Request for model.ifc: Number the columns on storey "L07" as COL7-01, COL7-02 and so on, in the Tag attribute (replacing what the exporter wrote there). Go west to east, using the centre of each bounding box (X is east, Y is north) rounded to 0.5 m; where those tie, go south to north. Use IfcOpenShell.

First a look at what the model holds.

```python
import ifcopenshell
import ifcopenshell.util.element
import ifcopenshell.util.placement

model = ifcopenshell.open("model.ifc")
print(model.schema)
storey = next(s for s in model.by_type("IfcBuildingStorey") if s.Name == "L07")
columns = [e for e in ifcopenshell.util.element.get_decomposition(storey) if e.is_a("IfcColumn")]
for e in sorted(columns, key=lambda e: e.id()):
    origin = ifcopenshell.util.placement.get_local_placement(e.ObjectPlacement)[:3, 3]
    print(e.id(), e.Tag, e.Name, origin.round(2) + 0.0, sep=" | ")
```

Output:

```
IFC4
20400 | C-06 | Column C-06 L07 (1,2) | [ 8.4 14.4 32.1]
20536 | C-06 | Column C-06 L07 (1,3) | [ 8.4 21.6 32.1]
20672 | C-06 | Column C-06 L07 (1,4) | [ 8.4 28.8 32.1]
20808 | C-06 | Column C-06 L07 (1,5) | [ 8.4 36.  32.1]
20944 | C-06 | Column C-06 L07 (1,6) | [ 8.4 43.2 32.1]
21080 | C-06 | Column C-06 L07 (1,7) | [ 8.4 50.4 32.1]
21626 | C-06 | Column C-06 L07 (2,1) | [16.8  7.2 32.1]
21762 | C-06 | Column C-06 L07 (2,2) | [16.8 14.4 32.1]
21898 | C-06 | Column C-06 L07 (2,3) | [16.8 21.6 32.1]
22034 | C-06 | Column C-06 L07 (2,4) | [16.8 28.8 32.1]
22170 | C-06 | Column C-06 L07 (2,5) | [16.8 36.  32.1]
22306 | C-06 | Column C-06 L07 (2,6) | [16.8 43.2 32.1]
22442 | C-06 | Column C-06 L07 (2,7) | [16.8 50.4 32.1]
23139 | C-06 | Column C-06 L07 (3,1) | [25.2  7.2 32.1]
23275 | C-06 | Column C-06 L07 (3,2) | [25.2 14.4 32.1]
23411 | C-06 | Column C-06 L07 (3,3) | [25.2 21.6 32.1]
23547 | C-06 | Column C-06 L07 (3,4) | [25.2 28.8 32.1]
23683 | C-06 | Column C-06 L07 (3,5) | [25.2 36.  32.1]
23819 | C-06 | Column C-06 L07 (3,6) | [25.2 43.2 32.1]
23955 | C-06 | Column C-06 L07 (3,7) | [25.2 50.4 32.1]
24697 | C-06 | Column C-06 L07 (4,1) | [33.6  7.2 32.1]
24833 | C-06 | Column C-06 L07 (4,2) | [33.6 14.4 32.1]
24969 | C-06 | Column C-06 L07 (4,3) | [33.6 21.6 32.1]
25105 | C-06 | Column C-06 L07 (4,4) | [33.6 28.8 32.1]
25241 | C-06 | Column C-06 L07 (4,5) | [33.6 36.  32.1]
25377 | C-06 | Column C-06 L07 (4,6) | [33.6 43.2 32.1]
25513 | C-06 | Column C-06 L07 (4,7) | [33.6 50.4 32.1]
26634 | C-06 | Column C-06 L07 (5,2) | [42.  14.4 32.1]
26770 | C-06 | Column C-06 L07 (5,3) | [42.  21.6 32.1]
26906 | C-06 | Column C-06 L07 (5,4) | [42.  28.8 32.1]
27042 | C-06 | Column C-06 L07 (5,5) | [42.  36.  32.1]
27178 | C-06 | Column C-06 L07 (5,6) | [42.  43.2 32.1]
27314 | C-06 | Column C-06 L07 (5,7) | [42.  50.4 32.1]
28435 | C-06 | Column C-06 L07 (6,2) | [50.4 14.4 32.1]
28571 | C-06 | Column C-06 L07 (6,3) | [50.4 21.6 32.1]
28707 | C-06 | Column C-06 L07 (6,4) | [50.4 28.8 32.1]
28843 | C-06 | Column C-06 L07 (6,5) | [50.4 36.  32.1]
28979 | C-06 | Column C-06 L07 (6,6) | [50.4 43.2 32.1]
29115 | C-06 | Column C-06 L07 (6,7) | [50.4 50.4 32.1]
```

```python
import ifcopenshell
import ifcopenshell.geom
import ifcopenshell.util.element
import ifcopenshell.util.shape

model = ifcopenshell.open("model.ifc")
settings = ifcopenshell.geom.settings()
settings.set("use-world-coords", True)


def centre(element):
    shape = ifcopenshell.geom.create_shape(settings, element)
    return ifcopenshell.util.shape.get_bbox_centroid(shape.geometry)


storey = next(s for s in model.by_type("IfcBuildingStorey") if s.Name == "L07")
columns = [e for e in ifcopenshell.util.element.get_decomposition(storey) if e.is_a("IfcColumn")]

# Insertion points can sit at a corner or the storey origin, so sort by the geometry (in metres).
centres = {e: centre(e) for e in columns}
columns.sort(key=lambda e: (round(centres[e][0] / 0.5), centres[e][1]))

for i, e in enumerate(columns, start=1):
    number = f"COL7-{i:02d}"
    e.Tag = number
    print(e.id(), number)

model.write("model_rev.ifc")
```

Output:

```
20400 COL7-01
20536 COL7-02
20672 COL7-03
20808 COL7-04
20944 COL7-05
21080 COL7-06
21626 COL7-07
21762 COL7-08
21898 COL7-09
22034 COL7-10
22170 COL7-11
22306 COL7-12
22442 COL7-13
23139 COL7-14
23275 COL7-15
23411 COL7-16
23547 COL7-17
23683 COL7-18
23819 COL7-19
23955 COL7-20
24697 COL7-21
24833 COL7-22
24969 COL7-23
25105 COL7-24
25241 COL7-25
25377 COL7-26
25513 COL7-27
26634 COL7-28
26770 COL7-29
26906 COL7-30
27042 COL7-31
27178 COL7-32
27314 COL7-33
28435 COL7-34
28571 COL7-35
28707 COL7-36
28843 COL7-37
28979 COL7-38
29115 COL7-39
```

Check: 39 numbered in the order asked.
